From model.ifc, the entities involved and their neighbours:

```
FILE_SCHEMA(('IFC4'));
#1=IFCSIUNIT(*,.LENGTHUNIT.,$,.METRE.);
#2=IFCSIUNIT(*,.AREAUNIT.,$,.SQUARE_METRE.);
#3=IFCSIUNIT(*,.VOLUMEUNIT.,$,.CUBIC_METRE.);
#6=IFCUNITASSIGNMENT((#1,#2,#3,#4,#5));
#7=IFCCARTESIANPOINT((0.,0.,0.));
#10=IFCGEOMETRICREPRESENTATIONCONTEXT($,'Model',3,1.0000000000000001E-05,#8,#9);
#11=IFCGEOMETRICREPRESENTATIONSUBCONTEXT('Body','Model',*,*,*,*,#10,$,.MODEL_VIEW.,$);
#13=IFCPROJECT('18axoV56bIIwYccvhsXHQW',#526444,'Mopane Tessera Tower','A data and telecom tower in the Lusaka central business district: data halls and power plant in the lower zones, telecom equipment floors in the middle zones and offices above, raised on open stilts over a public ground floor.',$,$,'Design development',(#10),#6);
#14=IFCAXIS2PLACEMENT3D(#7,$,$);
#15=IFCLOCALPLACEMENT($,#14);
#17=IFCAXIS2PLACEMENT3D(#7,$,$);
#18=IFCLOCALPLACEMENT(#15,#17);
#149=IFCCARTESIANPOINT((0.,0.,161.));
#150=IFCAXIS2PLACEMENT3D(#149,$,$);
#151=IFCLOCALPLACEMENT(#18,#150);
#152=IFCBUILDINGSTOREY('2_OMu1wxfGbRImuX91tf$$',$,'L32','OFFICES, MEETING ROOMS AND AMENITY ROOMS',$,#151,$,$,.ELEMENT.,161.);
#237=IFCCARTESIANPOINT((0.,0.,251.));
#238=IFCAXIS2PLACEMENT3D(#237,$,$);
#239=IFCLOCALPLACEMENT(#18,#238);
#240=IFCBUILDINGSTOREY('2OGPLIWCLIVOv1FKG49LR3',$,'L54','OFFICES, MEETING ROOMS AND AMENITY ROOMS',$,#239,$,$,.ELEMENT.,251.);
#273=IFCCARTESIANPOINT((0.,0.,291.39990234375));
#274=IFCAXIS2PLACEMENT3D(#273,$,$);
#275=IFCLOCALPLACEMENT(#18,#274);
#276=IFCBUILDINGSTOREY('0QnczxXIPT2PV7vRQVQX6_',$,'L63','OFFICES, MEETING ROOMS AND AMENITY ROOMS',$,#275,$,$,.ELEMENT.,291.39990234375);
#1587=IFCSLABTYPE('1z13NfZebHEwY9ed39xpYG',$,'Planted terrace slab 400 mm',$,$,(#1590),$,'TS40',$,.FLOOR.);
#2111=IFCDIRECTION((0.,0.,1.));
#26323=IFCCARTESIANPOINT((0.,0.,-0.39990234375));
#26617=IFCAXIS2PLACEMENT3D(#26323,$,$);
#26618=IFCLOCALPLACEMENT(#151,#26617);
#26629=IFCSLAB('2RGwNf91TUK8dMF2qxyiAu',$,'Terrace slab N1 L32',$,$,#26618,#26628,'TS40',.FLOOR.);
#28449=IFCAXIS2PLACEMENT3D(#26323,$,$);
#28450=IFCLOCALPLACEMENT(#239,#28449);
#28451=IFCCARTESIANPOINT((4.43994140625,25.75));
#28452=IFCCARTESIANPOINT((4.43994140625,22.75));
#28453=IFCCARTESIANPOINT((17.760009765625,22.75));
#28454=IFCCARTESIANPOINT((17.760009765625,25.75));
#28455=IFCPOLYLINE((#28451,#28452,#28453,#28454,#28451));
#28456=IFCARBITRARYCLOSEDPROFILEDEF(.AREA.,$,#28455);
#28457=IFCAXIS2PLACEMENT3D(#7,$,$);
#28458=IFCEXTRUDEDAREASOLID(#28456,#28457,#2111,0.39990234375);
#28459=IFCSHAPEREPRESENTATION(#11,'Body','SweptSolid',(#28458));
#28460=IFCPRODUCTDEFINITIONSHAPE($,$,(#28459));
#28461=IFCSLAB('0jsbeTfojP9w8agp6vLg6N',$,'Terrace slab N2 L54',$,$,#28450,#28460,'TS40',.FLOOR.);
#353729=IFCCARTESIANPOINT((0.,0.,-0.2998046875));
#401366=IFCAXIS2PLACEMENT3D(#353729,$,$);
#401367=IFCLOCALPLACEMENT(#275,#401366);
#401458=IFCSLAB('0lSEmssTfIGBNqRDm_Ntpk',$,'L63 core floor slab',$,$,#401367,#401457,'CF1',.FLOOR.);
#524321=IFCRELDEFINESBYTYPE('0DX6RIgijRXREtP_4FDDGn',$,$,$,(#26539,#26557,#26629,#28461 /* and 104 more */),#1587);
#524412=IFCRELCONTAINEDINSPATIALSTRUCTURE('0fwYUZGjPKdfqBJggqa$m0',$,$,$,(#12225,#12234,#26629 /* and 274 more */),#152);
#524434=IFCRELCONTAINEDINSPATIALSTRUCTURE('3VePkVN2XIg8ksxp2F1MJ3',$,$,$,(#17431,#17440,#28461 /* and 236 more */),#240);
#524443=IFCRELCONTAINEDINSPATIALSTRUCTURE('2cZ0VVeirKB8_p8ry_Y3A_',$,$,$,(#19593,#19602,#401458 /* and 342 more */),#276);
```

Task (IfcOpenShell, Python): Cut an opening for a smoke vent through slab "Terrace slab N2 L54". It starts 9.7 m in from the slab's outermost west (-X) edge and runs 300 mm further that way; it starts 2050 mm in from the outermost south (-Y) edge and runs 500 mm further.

```python
import numpy as np
import ifcopenshell
import ifcopenshell.api.feature
import ifcopenshell.api.geometry
import ifcopenshell.api.root
import ifcopenshell.geom
import ifcopenshell.util.placement
import ifcopenshell.util.representation
import ifcopenshell.util.shape
import ifcopenshell.util.unit

model = ifcopenshell.open("model.ifc")
unit_scale = ifcopenshell.util.unit.calculate_unit_scale(model)
settings = ifcopenshell.geom.settings()


def volume(element):
    """Net volume in cubic metres, openings subtracted."""
    shape = ifcopenshell.geom.create_shape(settings, element)
    return ifcopenshell.util.shape.get_volume(shape.geometry)


slab = model.by_guid("0jsbeTfojP9w8agp6vLg6N")
before = volume(slab)

# Extent in the slab's own axes, in metres. The edges named are its -X and -Y sides.
slab_shape = ifcopenshell.geom.create_shape(settings, slab)
vertices = ifcopenshell.util.shape.get_vertices(slab_shape.geometry)
x_min, y_min, bottom = vertices.min(axis=0)
top = vertices[:, 2].max()

opening = ifcopenshell.api.root.create_entity(model, ifc_class="IfcOpeningElement", name="Smoke vent opening", predefined_type="OPENING")
context = ifcopenshell.util.representation.get_context(model, "Model", "Body", "MODEL_VIEW")
width, depth = 0.3, 0.5
outline = [(0.0, 0.0), (width, 0.0), (width, depth), (0.0, depth), (0.0, 0.0)]
# Overshoot both faces by 50 mm so the cut is clean.
shape = ifcopenshell.api.geometry.add_slab_representation(
    model, context=context, depth=top - bottom + 0.1, polyline=outline
)
ifcopenshell.api.geometry.assign_representation(model, product=opening, representation=shape)

matrix = ifcopenshell.util.placement.get_local_placement(slab.ObjectPlacement)
matrix[:, 3] = matrix @ np.append(np.array([x_min + 9.7, y_min + 2.05, bottom - 0.05]) / unit_scale, 1.0)
ifcopenshell.api.geometry.edit_object_placement(model, product=opening, matrix=matrix, is_si=False)
ifcopenshell.api.feature.add_feature(model, feature=opening, element=slab)

after = volume(slab)

print(f"slab volume {before:.3f} -> {after:.3f} m3")

model.write("model_rev.ifc")
```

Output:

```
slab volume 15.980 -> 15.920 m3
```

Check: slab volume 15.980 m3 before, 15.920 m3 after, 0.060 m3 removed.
